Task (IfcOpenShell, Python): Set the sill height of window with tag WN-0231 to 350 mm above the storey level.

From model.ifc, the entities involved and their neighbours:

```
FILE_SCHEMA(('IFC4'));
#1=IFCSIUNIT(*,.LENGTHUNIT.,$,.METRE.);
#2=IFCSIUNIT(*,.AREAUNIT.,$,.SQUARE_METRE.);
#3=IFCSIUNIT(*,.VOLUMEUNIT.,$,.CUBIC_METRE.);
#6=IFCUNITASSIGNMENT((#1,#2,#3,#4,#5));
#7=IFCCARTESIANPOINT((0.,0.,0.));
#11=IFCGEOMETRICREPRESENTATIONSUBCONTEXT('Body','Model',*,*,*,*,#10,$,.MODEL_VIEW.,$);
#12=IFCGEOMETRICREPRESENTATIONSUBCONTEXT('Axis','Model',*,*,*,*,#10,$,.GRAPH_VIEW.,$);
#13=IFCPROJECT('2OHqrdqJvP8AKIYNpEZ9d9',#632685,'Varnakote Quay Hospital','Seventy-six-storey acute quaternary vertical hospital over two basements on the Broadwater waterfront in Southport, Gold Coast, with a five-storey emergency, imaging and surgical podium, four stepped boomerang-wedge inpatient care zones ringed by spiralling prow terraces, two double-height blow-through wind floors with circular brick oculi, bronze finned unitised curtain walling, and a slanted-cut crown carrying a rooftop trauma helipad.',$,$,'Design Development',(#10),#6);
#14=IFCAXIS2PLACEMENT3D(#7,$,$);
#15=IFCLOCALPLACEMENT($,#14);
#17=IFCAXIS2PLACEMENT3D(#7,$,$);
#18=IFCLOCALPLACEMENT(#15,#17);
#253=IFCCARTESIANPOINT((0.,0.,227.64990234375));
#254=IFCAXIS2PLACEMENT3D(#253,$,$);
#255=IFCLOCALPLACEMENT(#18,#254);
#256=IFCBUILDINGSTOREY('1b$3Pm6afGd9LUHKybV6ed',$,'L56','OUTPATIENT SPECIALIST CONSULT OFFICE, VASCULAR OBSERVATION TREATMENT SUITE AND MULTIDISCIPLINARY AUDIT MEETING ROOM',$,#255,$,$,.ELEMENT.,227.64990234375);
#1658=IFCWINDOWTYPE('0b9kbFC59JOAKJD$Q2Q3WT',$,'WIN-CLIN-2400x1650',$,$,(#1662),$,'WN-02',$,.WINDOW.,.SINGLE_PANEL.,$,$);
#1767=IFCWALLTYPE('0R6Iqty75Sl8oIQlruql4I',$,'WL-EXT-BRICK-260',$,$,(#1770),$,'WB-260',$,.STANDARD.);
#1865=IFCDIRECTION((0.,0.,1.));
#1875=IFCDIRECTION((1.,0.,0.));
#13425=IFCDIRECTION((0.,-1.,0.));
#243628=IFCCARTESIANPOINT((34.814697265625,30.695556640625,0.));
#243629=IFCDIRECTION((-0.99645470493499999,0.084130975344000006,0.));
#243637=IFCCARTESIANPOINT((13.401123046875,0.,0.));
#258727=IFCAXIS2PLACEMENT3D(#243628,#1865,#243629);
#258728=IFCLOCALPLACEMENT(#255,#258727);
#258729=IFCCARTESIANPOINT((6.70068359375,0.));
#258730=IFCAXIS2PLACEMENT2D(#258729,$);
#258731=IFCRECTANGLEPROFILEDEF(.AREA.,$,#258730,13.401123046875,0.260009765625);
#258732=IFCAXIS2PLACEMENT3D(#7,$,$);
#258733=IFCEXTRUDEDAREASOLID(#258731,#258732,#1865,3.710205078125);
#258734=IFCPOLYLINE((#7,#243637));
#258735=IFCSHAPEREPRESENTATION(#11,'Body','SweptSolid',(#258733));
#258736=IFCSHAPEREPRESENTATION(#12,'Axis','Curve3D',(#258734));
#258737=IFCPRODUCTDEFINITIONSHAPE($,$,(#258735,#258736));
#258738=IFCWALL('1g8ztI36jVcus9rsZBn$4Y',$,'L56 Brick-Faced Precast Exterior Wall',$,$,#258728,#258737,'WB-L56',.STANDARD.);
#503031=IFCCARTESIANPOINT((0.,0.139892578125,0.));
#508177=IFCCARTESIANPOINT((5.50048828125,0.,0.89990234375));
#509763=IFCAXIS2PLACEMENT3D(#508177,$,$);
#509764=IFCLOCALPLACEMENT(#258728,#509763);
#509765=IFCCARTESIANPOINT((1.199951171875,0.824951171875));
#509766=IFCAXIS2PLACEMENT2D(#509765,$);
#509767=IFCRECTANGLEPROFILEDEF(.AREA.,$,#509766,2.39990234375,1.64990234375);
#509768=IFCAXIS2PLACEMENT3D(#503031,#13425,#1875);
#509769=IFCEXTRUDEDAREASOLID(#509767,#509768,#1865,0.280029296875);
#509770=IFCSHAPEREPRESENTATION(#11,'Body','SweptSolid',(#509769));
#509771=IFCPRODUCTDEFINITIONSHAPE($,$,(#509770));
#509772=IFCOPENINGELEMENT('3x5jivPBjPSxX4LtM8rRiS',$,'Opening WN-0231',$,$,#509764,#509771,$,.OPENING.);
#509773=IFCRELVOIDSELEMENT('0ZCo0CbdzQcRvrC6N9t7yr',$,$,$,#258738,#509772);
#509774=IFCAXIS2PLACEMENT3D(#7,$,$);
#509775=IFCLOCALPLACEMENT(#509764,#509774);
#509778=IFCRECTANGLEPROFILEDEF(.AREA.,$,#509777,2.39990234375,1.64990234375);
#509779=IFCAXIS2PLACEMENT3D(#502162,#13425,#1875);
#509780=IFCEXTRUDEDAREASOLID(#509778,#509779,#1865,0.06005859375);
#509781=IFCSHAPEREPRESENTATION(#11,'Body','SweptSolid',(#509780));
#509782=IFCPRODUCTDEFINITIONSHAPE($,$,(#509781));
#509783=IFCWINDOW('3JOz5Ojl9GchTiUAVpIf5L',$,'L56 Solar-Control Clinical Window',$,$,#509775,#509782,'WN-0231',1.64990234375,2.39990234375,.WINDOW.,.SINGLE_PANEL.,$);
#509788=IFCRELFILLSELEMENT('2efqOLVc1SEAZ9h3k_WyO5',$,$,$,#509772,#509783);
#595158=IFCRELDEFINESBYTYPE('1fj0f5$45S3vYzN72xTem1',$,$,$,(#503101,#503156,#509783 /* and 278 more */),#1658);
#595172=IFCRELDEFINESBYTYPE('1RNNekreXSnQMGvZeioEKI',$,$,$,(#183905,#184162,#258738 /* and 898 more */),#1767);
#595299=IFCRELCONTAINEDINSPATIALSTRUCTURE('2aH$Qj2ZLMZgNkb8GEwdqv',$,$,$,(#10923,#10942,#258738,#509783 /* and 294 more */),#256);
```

```python
import numpy as np
import ifcopenshell
import ifcopenshell.api.geometry
import ifcopenshell.geom
import ifcopenshell.util.element
import ifcopenshell.util.placement
import ifcopenshell.util.shape
import ifcopenshell.util.unit

model = ifcopenshell.open("model.ifc")
unit_scale = ifcopenshell.util.unit.calculate_unit_scale(model)

window = model.by_guid("3JOz5Ojl9GchTiUAVpIf5L")
opening = window.FillsVoids[0].RelatingOpeningElement
storey = ifcopenshell.util.element.get_container(window, ifc_class="IfcBuildingStorey")
level = ifcopenshell.util.placement.get_local_placement(storey.ObjectPlacement)[2, 3]

# The opening's origin need not be at the sill, so measure its lowest point.
shape = ifcopenshell.geom.create_shape(ifcopenshell.geom.settings(), opening)
bottom = ifcopenshell.util.shape.get_shape_bottom_elevation(shape, shape.geometry) / unit_scale
dz = level + 0.35 / unit_scale - bottom

shift = np.array([0.0, 0.0, dz])
# The window is placed relative to its opening, so it follows when the opening moves.
matrix = ifcopenshell.util.placement.get_local_placement(opening.ObjectPlacement)
matrix[:3, 3] += shift
ifcopenshell.api.geometry.edit_object_placement(
    model, product=opening, matrix=matrix, is_si=False, should_transform_children=True
)

print(f"moved by {dz * unit_scale:+.3f} m")

model.write("model_rev.ifc")
```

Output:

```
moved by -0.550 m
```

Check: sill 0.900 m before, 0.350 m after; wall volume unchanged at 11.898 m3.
